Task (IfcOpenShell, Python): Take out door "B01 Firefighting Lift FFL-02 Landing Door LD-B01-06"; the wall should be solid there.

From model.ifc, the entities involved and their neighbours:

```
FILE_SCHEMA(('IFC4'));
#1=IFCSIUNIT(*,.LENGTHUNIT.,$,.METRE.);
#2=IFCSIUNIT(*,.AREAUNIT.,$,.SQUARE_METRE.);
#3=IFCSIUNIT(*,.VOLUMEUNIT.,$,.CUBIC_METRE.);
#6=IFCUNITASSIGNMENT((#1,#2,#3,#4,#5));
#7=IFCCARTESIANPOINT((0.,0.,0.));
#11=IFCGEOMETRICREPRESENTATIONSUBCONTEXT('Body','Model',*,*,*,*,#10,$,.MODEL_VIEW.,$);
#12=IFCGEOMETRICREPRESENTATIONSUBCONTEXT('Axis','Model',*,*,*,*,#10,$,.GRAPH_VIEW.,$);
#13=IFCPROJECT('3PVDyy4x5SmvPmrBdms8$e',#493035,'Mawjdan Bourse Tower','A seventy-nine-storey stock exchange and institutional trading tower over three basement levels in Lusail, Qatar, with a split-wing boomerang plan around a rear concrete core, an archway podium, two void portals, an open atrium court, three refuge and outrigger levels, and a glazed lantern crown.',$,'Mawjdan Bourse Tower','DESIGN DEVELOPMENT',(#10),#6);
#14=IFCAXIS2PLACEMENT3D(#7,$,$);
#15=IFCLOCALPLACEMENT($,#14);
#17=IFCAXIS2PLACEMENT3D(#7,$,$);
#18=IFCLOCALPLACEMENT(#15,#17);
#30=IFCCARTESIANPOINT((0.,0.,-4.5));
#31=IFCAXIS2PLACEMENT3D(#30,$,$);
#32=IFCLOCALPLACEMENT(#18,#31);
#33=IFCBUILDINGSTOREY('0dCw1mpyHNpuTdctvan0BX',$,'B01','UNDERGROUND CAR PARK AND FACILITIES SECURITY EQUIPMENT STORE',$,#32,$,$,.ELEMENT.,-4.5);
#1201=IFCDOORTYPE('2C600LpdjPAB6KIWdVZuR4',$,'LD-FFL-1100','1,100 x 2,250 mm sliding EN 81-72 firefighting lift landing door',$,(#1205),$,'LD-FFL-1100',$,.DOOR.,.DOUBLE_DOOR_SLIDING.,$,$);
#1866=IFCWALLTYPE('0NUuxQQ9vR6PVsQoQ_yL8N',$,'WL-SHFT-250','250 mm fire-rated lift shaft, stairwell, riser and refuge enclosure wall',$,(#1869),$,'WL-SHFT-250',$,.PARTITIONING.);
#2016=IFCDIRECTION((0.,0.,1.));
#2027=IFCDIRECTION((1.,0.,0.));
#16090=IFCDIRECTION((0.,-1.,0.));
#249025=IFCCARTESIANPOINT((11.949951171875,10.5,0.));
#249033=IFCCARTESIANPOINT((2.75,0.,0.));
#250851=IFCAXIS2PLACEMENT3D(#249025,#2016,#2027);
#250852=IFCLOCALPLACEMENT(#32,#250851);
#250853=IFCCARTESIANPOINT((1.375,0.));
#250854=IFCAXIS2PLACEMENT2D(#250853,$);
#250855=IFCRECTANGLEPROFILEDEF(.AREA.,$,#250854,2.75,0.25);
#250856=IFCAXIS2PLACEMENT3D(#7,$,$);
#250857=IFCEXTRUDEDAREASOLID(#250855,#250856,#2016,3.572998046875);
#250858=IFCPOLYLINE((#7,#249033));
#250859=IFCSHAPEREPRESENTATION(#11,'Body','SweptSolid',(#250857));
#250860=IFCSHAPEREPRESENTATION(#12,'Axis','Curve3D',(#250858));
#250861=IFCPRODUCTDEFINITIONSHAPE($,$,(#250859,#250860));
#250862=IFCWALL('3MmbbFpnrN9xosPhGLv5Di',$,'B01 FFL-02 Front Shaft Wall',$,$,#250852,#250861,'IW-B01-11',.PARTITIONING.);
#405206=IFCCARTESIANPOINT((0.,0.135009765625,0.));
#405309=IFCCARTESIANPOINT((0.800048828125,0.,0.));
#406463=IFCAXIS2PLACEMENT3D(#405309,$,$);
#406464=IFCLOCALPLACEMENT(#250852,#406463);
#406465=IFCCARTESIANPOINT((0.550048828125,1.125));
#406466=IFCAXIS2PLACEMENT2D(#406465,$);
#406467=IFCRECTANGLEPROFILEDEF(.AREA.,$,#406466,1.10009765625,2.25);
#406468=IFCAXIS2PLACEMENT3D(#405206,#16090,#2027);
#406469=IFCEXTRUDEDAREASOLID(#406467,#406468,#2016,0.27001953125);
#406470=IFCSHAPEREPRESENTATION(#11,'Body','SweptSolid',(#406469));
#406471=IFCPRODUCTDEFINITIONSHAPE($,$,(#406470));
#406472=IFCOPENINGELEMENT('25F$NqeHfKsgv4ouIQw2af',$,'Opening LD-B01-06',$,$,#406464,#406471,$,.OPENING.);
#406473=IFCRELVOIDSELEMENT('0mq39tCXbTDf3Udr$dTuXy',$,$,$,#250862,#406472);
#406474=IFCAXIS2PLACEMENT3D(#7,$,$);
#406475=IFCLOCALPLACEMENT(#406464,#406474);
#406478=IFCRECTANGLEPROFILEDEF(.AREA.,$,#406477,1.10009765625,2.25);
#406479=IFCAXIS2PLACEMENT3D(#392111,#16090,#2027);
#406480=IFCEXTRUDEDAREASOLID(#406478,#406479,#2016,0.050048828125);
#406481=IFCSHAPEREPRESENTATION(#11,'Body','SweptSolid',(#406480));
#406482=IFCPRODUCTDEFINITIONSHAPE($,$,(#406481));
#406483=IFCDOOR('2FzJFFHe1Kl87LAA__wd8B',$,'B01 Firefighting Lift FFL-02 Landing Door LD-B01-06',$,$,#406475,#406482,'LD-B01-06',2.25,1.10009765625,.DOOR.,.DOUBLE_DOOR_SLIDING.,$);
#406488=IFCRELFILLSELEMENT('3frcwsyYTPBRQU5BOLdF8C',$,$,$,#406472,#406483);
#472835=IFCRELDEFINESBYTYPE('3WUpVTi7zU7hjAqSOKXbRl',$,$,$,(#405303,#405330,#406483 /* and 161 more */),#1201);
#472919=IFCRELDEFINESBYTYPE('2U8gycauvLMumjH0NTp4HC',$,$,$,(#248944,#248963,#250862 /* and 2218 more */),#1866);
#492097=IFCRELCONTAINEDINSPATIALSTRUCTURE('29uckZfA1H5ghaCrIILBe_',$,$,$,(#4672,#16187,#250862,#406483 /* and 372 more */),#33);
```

```python
import ifcopenshell
import ifcopenshell.api.feature
import ifcopenshell.api.root
import ifcopenshell.geom
import ifcopenshell.util.shape

model = ifcopenshell.open("model.ifc")
settings = ifcopenshell.geom.settings()


def volume(element):
    """Net volume in cubic metres, openings subtracted."""
    shape = ifcopenshell.geom.create_shape(settings, element)
    return ifcopenshell.util.shape.get_volume(shape.geometry)


door = model.by_id(406483)
opening = door.FillsVoids[0].RelatingOpeningElement
wall = opening.VoidsElements[0].RelatingBuildingElement
before = volume(wall)

ifcopenshell.api.root.remove_product(model, product=door)
ifcopenshell.api.feature.remove_feature(model, feature=opening)

after = volume(wall)

print(f"wall volume {before:.3f} -> {after:.3f} m3")

model.write("model-out.ifc")
```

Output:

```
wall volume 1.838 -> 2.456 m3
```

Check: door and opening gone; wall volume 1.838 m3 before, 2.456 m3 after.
